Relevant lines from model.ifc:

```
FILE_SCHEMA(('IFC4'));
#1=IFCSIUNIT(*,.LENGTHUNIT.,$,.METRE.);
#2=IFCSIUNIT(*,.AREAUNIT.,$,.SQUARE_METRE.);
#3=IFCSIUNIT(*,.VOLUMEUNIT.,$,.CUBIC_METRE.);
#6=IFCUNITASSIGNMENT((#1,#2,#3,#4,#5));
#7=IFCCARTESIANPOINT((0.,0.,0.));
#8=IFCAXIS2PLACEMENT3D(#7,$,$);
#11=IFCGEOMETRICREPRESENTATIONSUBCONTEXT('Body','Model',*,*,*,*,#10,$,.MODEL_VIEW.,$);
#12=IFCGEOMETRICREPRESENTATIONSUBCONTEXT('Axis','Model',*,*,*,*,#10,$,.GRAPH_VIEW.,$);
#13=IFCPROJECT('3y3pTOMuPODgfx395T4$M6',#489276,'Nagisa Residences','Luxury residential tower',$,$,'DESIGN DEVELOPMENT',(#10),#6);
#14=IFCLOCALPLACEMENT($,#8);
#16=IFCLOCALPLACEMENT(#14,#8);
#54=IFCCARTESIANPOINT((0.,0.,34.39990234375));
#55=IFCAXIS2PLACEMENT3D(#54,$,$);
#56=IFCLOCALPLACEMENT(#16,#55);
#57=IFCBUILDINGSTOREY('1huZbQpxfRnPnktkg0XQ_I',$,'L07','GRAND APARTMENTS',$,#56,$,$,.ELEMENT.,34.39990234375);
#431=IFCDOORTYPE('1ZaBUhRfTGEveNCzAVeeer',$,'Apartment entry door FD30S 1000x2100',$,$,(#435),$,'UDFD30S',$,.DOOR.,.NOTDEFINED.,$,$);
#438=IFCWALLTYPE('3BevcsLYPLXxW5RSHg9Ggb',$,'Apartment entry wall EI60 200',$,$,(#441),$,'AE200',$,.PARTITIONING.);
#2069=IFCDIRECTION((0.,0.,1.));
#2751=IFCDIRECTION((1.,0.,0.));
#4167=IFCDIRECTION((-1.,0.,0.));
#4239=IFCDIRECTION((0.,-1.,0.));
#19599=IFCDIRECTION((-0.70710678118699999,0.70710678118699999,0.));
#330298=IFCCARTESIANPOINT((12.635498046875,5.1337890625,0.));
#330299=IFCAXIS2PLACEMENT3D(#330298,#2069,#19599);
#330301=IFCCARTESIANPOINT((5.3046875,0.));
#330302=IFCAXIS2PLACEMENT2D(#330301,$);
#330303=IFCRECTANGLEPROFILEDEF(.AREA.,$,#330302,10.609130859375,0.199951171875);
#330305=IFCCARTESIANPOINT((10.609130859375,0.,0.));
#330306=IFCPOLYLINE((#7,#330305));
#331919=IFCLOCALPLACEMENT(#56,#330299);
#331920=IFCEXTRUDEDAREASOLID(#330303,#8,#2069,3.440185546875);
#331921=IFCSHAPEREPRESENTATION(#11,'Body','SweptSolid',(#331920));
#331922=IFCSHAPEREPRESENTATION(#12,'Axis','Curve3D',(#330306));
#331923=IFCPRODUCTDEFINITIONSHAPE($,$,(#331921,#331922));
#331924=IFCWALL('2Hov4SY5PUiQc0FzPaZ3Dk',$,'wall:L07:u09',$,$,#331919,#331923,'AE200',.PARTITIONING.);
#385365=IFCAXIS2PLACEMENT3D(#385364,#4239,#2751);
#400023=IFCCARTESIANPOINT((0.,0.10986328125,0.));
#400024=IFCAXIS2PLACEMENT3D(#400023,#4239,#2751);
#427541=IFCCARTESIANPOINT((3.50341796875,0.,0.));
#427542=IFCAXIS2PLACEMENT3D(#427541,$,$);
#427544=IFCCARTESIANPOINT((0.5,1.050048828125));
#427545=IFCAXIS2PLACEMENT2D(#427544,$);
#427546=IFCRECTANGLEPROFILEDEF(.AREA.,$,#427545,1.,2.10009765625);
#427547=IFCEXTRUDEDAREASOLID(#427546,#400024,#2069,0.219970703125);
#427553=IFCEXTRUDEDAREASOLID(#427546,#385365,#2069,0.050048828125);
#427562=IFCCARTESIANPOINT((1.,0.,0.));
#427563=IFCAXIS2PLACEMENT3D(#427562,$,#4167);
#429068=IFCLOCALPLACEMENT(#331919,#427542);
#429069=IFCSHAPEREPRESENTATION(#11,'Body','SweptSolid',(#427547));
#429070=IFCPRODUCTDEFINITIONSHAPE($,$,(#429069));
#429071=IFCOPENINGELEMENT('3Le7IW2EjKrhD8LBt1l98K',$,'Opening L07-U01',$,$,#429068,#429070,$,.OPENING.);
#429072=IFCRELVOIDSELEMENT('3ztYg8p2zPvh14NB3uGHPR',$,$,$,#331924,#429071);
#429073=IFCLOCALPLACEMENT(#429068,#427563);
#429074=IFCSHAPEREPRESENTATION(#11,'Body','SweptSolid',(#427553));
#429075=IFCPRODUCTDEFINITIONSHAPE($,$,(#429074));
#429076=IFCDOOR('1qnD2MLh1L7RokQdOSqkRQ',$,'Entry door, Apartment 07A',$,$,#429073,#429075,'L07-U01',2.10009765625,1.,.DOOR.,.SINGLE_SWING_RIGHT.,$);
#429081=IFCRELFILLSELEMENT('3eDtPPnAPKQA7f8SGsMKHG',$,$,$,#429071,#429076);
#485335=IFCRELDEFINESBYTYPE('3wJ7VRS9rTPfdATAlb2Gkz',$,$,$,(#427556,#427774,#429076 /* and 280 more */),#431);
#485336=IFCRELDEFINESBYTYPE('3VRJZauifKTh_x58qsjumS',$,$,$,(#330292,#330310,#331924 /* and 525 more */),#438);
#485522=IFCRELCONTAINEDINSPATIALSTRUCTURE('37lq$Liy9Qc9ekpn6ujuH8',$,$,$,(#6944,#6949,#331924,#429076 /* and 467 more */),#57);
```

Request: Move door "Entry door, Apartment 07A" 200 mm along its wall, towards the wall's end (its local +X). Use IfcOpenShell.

```python
import ifcopenshell
import ifcopenshell.api.geometry
import ifcopenshell.util.placement
import ifcopenshell.util.unit

model = ifcopenshell.open("model.ifc")
unit_scale = ifcopenshell.util.unit.calculate_unit_scale(model)

door = model.by_guid("1qnD2MLh1L7RokQdOSqkRQ")
opening = door.FillsVoids[0].RelatingOpeningElement
wall = opening.VoidsElements[0].RelatingBuildingElement

wall_matrix = ifcopenshell.util.placement.get_local_placement(wall.ObjectPlacement)
shift = wall_matrix[:3, 0] * 0.2 / unit_scale
before = ifcopenshell.util.placement.get_local_placement(door.ObjectPlacement)[:3, 3].copy()

# The door is placed relative to its opening, so it follows when the opening moves.
matrix = ifcopenshell.util.placement.get_local_placement(opening.ObjectPlacement)
matrix[:3, 3] += shift
ifcopenshell.api.geometry.edit_object_placement(
    model, product=opening, matrix=matrix, is_si=False, should_transform_children=True
)

after = ifcopenshell.util.placement.get_local_placement(door.ObjectPlacement)[:3, 3]
print("door moved by", (after - before).round(3) + 0.0)

model.write("model_edited.ifc")
```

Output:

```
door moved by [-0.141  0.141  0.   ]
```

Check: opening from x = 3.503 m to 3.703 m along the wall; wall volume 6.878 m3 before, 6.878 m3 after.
